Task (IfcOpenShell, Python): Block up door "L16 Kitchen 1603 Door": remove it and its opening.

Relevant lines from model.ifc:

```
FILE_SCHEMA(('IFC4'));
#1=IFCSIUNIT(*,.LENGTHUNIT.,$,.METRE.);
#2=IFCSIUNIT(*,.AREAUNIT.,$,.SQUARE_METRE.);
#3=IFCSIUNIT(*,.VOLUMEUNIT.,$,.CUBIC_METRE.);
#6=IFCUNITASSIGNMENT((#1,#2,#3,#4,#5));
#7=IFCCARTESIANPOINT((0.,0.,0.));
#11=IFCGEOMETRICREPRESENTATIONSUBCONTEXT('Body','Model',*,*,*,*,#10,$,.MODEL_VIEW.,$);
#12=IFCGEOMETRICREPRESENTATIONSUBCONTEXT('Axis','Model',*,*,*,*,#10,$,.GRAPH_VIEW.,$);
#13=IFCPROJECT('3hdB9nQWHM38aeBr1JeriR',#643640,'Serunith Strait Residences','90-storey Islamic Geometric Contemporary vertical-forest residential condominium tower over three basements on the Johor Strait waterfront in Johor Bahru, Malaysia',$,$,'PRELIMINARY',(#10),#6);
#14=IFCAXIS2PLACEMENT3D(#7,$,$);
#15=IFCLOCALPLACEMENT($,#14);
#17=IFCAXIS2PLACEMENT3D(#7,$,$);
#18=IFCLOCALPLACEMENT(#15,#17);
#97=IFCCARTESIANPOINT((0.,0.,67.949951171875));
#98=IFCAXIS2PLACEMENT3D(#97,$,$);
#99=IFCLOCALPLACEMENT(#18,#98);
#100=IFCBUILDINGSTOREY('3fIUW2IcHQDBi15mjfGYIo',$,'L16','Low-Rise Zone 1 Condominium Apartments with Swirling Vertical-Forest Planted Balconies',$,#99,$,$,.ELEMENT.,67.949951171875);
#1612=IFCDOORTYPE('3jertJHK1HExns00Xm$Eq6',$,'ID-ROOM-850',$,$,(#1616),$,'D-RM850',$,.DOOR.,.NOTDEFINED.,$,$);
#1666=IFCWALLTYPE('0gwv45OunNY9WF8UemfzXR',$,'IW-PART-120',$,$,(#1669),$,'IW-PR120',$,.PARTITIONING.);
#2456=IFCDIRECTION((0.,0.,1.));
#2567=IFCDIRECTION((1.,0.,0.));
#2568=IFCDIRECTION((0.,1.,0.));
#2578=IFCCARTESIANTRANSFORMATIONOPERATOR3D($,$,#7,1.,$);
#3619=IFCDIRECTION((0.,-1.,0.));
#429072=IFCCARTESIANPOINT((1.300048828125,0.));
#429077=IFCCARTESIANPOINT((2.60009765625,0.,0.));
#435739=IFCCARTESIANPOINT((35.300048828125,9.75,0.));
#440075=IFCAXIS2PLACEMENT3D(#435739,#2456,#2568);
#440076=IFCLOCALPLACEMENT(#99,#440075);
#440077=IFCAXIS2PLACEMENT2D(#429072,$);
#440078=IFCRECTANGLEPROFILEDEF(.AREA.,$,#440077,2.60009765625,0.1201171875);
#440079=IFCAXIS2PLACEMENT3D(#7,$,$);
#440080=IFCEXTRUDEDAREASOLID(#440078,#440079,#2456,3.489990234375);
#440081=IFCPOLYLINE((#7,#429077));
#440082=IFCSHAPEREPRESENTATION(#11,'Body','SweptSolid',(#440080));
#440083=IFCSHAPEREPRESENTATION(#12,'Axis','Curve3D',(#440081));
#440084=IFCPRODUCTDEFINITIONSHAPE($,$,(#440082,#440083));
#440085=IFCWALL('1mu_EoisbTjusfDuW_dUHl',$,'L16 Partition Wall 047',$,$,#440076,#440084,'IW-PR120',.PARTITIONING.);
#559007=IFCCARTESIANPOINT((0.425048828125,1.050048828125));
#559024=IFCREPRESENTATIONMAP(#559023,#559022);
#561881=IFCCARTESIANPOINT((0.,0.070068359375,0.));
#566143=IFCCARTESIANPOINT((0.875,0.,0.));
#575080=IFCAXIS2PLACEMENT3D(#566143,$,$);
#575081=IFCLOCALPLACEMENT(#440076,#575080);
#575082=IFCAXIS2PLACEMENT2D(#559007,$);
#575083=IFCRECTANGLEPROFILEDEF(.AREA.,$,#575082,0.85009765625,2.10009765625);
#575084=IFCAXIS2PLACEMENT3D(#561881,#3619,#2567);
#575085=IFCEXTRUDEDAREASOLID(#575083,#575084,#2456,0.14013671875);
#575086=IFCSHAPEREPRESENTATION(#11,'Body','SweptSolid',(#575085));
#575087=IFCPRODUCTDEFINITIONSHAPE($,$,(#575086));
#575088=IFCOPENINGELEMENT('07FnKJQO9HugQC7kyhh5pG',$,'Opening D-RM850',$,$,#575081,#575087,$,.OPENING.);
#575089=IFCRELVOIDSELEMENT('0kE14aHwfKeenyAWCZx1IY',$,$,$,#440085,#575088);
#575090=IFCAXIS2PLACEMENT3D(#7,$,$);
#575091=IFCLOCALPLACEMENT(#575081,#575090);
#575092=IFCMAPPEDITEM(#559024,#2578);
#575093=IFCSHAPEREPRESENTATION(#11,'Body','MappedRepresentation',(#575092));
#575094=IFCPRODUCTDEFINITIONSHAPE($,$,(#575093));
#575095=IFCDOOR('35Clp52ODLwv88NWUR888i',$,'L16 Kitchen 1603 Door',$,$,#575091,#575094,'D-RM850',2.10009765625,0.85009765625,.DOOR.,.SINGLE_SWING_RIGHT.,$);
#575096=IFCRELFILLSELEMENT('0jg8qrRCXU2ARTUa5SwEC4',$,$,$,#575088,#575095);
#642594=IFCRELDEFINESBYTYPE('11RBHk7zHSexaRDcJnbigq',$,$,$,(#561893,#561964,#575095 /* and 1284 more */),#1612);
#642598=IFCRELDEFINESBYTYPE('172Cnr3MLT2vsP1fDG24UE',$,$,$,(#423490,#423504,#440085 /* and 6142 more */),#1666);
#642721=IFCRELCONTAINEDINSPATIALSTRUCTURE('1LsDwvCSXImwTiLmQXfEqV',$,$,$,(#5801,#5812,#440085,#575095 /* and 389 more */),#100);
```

```python
import ifcopenshell
import ifcopenshell.api.feature
import ifcopenshell.api.root
import ifcopenshell.geom
import ifcopenshell.util.shape

model = ifcopenshell.open("model.ifc")
settings = ifcopenshell.geom.settings()


def volume(element):
    """Net volume in cubic metres, openings subtracted."""
    shape = ifcopenshell.geom.create_shape(settings, element)
    return ifcopenshell.util.shape.get_volume(shape.geometry)


door = model.by_guid("35Clp52ODLwv88NWUR888i")
opening = door.FillsVoids[0].RelatingOpeningElement
wall = opening.VoidsElements[0].RelatingBuildingElement
before = volume(wall)

ifcopenshell.api.root.remove_product(model, product=door)
ifcopenshell.api.feature.remove_feature(model, feature=opening)

after = volume(wall)

print(f"wall volume {before:.3f} -> {after:.3f} m3")

model.write("model-out.ifc")
```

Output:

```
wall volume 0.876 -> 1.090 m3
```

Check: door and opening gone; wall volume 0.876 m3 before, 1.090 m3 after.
